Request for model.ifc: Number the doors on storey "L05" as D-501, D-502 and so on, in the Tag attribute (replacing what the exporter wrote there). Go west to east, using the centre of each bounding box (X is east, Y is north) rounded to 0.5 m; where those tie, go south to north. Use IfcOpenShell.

First a look at what the model holds.

```python
import ifcopenshell
import ifcopenshell.util.element
import ifcopenshell.util.placement

model = ifcopenshell.open("model.ifc")
print(model.schema)
storey = next(s for s in model.by_type("IfcBuildingStorey") if s.Name == "L05")
doors = [e for e in ifcopenshell.util.element.get_decomposition(storey) if e.is_a("IfcDoor")]
for e in sorted(doors, key=lambda e: e.id()):
    origin = ifcopenshell.util.placement.get_local_placement(e.ObjectPlacement)[:3, 3]
    print(e.id(), e.Tag, e.Name, origin.round(2) + 0.0, sep=" | ")
```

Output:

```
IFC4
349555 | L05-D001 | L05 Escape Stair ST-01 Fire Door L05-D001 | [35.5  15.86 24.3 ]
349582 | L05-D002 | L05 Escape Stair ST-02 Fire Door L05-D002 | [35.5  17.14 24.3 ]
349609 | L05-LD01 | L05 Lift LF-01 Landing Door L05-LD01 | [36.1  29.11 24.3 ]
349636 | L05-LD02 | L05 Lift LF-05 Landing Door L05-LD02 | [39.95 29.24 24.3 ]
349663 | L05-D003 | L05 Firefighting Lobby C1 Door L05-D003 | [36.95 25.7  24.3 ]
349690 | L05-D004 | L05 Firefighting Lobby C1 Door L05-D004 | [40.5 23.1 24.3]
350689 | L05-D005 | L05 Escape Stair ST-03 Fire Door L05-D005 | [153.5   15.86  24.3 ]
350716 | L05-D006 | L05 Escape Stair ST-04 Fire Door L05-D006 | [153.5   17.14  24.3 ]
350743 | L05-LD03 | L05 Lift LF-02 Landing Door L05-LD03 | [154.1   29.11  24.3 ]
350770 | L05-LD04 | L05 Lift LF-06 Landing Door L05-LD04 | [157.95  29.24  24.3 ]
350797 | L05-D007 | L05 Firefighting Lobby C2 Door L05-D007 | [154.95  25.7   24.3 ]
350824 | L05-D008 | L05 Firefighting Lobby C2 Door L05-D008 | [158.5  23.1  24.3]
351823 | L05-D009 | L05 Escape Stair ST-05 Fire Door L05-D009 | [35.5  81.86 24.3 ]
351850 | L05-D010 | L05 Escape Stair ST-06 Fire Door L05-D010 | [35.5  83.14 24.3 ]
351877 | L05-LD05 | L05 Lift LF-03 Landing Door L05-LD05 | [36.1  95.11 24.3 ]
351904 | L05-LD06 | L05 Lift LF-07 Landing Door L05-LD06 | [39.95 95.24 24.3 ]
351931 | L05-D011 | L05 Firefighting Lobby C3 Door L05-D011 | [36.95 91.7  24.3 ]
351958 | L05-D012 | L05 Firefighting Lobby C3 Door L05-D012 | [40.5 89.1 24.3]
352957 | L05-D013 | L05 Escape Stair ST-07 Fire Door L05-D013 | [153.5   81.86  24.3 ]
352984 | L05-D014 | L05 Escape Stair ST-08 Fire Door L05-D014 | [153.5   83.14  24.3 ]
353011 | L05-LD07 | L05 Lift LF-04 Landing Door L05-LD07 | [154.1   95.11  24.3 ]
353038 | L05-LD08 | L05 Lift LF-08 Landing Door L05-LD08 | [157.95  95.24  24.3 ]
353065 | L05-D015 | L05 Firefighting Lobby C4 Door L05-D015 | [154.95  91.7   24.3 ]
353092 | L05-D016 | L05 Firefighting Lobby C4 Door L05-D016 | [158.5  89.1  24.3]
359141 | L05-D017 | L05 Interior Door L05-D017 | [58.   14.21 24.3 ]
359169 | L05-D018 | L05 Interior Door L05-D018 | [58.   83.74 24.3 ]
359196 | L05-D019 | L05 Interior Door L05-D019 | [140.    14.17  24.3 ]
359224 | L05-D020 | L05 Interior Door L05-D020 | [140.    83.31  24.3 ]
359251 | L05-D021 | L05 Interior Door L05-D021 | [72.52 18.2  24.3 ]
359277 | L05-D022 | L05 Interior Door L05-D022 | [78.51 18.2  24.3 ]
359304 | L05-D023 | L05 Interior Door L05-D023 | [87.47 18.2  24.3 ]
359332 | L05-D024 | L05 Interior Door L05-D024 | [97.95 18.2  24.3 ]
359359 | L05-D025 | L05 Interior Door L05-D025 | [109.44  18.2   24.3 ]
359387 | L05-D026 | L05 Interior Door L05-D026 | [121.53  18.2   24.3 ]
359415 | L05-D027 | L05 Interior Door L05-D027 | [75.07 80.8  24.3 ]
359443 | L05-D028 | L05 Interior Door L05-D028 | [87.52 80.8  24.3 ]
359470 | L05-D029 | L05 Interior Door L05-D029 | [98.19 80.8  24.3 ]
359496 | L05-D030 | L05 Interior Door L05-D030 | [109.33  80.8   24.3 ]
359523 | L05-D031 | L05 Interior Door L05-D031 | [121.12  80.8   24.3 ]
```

```python
import ifcopenshell
import ifcopenshell.geom
import ifcopenshell.util.element
import ifcopenshell.util.shape

model = ifcopenshell.open("model.ifc")
settings = ifcopenshell.geom.settings()
settings.set("use-world-coords", True)


def centre(element):
    shape = ifcopenshell.geom.create_shape(settings, element)
    return ifcopenshell.util.shape.get_bbox_centroid(shape.geometry)


storey = next(s for s in model.by_type("IfcBuildingStorey") if s.Name == "L05")
doors = [e for e in ifcopenshell.util.element.get_decomposition(storey) if e.is_a("IfcDoor")]

# Insertion points can sit at a corner or the storey origin, so sort by the geometry (in metres).
centres = {e: centre(e) for e in doors}
doors.sort(key=lambda e: (round(centres[e][0] / 0.5), centres[e][1]))

for i, e in enumerate(doors, start=1):
    number = f"D-5{i:02d}"
    e.Tag = number
    print(e.id(), number)

model.write("model_rev.ifc")
```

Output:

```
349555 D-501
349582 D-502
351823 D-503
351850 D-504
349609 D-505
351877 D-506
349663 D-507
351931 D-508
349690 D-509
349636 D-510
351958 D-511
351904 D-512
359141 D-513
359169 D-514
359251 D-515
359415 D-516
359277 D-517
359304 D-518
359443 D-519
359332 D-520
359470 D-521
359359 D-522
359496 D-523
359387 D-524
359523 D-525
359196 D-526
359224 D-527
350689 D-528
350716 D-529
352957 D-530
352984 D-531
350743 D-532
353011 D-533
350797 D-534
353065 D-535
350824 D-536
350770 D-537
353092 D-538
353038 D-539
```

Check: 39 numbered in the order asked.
